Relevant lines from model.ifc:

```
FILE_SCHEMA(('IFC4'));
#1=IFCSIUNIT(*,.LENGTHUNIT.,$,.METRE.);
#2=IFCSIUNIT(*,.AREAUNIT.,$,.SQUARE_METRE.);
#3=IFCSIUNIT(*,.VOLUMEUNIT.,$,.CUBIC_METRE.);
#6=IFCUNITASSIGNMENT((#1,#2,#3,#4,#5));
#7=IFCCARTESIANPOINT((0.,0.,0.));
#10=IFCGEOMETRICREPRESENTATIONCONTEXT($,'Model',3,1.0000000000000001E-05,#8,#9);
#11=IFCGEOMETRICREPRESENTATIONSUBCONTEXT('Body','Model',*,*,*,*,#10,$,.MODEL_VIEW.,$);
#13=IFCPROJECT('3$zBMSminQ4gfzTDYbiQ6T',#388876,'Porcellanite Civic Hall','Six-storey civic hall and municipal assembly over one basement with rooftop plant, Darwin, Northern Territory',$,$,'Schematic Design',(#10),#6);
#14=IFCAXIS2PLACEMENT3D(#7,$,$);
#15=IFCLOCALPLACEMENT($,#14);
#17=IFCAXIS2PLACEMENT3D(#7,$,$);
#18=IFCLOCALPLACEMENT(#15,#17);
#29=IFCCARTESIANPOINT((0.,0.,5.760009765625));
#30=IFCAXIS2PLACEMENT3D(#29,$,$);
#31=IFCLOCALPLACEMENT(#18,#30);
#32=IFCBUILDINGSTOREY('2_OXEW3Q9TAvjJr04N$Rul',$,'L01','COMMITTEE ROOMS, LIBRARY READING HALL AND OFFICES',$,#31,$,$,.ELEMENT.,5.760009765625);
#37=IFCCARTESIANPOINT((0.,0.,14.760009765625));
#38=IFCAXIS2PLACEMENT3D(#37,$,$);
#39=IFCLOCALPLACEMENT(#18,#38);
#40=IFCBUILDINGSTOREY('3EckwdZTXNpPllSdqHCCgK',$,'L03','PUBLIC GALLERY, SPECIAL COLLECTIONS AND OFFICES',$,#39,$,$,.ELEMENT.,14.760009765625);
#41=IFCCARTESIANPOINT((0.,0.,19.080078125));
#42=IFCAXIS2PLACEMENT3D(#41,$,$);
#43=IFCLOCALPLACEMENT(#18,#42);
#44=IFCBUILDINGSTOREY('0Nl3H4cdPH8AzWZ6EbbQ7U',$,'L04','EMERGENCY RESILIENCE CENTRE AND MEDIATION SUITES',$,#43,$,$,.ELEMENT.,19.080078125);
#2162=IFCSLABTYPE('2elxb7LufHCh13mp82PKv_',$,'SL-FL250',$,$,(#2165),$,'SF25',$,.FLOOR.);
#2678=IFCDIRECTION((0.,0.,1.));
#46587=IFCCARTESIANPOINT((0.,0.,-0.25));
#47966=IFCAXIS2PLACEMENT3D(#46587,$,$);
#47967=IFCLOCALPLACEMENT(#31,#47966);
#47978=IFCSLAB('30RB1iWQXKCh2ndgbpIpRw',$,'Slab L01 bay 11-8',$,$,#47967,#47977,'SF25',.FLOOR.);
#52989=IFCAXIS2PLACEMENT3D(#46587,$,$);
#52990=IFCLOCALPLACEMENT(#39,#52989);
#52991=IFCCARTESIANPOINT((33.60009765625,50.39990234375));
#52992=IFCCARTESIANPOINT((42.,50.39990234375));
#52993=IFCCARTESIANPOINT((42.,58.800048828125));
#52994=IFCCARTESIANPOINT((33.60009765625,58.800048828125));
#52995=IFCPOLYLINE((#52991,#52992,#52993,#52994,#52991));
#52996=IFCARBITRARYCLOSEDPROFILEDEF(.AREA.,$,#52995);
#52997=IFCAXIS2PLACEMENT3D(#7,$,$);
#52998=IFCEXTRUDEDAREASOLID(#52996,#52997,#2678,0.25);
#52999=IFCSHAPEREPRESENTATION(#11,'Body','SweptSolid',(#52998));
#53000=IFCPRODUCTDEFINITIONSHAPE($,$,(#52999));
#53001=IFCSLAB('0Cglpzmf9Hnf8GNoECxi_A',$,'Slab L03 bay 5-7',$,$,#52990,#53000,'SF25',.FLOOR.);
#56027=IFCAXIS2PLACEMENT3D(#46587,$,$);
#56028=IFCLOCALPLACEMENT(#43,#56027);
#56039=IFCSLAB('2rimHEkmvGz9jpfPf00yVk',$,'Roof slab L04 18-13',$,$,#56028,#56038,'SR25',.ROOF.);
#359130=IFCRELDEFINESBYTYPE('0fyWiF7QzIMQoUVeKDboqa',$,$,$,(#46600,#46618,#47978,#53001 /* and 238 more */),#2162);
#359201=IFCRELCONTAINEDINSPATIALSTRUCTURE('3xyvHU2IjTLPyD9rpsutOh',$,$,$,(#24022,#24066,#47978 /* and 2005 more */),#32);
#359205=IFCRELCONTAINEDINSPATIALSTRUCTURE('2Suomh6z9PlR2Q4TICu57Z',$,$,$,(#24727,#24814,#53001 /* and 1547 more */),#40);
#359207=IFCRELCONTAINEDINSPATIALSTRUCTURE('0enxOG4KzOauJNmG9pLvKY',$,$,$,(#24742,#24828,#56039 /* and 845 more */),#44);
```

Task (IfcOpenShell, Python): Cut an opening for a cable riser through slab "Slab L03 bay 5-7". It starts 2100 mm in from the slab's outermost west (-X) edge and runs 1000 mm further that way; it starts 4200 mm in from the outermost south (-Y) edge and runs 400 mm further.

```python
import numpy as np
import ifcopenshell
import ifcopenshell.api.feature
import ifcopenshell.api.geometry
import ifcopenshell.api.root
import ifcopenshell.geom
import ifcopenshell.util.placement
import ifcopenshell.util.representation
import ifcopenshell.util.shape
import ifcopenshell.util.unit

model = ifcopenshell.open("model.ifc")
unit_scale = ifcopenshell.util.unit.calculate_unit_scale(model)
settings = ifcopenshell.geom.settings()


def volume(element):
    """Net volume in cubic metres, openings subtracted."""
    shape = ifcopenshell.geom.create_shape(settings, element)
    return ifcopenshell.util.shape.get_volume(shape.geometry)


slab = model.by_id(53001)
before = volume(slab)

# Extent in the slab's own axes, in metres. The edges named are its -X and -Y sides.
slab_shape = ifcopenshell.geom.create_shape(settings, slab)
vertices = ifcopenshell.util.shape.get_vertices(slab_shape.geometry)
x_min, y_min, bottom = vertices.min(axis=0)
top = vertices[:, 2].max()

opening = ifcopenshell.api.root.create_entity(model, ifc_class="IfcOpeningElement", name="Cable riser opening", predefined_type="OPENING")
context = ifcopenshell.util.representation.get_context(model, "Model", "Body", "MODEL_VIEW")
width, depth = 1, 0.4
outline = [(0.0, 0.0), (width, 0.0), (width, depth), (0.0, depth), (0.0, 0.0)]
# Overshoot both faces by 50 mm so the cut is clean.
shape = ifcopenshell.api.geometry.add_slab_representation(
    model, context=context, depth=top - bottom + 0.1, polyline=outline
)
ifcopenshell.api.geometry.assign_representation(model, product=opening, representation=shape)

matrix = ifcopenshell.util.placement.get_local_placement(slab.ObjectPlacement)
matrix[:, 3] = matrix @ np.append(np.array([x_min + 2.1, y_min + 4.2, bottom - 0.05]) / unit_scale, 1.0)
ifcopenshell.api.geometry.edit_object_placement(model, product=opening, matrix=matrix, is_si=False)
ifcopenshell.api.feature.add_feature(model, feature=opening, element=slab)

after = volume(slab)

print(f"slab volume {before:.3f} -> {after:.3f} m3")

model.write("model_v2.ifc")
```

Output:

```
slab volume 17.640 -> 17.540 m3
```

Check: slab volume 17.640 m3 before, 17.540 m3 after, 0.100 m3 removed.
